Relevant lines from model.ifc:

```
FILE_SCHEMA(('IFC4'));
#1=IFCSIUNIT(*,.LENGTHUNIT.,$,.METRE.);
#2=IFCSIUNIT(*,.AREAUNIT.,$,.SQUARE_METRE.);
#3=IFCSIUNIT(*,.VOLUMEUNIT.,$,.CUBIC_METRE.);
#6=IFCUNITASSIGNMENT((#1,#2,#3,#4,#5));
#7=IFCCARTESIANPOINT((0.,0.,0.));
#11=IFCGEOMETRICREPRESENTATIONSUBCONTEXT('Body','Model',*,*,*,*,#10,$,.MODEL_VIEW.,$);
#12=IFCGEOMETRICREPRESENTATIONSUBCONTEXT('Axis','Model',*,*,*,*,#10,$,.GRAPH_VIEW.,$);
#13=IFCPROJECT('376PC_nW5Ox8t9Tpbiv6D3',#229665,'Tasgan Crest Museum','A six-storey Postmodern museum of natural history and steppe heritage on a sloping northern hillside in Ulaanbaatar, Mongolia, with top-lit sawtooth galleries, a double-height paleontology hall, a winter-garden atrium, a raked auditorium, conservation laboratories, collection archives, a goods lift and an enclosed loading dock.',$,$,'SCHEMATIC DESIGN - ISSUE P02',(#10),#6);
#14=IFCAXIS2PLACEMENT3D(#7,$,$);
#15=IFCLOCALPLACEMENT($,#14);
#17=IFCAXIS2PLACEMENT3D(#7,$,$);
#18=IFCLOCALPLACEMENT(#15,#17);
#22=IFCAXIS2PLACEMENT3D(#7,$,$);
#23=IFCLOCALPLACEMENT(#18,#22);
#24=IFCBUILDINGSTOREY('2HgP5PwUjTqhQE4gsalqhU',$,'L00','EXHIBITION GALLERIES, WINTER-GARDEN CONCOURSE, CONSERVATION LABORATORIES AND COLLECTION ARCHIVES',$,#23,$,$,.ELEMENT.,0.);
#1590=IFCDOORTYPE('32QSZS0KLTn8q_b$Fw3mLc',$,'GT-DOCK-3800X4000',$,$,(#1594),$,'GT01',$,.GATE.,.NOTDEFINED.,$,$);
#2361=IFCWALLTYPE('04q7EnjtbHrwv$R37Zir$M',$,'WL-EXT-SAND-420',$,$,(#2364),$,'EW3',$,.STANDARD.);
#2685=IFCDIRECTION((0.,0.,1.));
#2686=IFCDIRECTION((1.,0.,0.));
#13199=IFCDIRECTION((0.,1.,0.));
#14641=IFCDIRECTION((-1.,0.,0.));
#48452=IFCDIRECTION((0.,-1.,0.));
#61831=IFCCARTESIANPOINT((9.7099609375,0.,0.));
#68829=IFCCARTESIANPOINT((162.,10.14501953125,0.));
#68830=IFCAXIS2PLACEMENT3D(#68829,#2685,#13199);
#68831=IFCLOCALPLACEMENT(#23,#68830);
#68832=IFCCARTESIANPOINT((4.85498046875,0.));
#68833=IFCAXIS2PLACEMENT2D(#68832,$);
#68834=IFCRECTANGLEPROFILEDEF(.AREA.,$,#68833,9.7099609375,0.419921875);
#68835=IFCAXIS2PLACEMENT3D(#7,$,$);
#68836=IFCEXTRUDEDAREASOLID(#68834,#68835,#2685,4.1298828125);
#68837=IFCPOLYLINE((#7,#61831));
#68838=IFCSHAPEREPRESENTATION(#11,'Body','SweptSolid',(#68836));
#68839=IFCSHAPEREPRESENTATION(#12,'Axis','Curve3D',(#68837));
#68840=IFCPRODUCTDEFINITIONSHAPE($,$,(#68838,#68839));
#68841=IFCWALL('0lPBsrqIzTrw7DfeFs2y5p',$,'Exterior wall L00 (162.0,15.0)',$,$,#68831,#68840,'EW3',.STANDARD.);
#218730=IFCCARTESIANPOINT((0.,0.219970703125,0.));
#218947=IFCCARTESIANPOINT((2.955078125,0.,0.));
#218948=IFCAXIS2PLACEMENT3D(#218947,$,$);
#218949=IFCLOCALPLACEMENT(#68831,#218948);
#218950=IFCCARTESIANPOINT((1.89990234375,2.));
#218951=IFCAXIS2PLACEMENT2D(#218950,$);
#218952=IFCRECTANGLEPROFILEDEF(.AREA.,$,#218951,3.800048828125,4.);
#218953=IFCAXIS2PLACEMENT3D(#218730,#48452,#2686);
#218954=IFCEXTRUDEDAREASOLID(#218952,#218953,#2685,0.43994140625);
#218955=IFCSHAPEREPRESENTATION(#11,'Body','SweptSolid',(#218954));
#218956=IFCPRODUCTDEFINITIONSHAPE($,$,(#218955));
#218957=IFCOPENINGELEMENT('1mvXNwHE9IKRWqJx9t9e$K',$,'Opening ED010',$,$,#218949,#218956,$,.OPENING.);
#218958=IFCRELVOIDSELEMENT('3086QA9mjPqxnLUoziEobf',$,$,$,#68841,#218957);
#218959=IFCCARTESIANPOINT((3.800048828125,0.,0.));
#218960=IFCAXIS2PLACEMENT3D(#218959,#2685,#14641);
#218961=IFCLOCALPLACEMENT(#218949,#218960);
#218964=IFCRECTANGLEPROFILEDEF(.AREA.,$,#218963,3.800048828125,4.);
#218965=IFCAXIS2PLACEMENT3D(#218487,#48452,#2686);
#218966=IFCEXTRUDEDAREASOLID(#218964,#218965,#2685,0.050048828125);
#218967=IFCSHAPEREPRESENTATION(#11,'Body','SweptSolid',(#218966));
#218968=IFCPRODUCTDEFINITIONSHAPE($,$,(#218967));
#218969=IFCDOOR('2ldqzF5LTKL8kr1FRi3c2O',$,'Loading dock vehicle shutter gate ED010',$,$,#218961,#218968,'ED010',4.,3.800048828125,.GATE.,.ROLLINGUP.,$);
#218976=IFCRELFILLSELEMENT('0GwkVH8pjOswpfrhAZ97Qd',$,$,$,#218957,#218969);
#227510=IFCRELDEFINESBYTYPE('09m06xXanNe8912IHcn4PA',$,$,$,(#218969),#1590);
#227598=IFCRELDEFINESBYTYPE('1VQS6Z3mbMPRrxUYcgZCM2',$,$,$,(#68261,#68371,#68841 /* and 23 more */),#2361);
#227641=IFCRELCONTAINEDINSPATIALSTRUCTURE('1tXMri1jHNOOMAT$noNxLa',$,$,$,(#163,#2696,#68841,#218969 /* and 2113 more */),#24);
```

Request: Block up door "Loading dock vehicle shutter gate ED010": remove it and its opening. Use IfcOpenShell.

```python
import ifcopenshell
import ifcopenshell.api.feature
import ifcopenshell.api.root
import ifcopenshell.geom
import ifcopenshell.util.shape

model = ifcopenshell.open("model.ifc")
settings = ifcopenshell.geom.settings()


def volume(element):
    """Net volume in cubic metres, openings subtracted."""
    shape = ifcopenshell.geom.create_shape(settings, element)
    return ifcopenshell.util.shape.get_volume(shape.geometry)


door = model.by_id(218969)
opening = door.FillsVoids[0].RelatingOpeningElement
wall = opening.VoidsElements[0].RelatingBuildingElement
before = volume(wall)

ifcopenshell.api.root.remove_product(model, product=door)
ifcopenshell.api.feature.remove_feature(model, feature=opening)

after = volume(wall)

print(f"wall volume {before:.3f} -> {after:.3f} m3")

model.write("model-out.ifc")
```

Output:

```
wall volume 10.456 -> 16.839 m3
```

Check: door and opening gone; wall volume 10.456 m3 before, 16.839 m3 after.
